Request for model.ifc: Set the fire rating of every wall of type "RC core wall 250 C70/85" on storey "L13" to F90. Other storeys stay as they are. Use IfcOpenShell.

First a look at what the model holds.

```python
import ifcopenshell
import ifcopenshell.util.element

model = ifcopenshell.open("model.ifc")
print(model.schema)
storey = next(s for s in model.by_type("IfcBuildingStorey") if s.Name == "L13")
walls = [e for e in ifcopenshell.util.element.get_decomposition(storey) if e.is_a("IfcWall")]
seen = {}
for e in walls:
    element_type = ifcopenshell.util.element.get_type(e)
    key = (element_type.Name if element_type != e and element_type else None, ifcopenshell.util.element.get_pset(e, "Pset_WallCommon", "FireRating"))
    seen[key] = seen.get(key, 0) + 1
for (name, value), count in sorted(seen.items(), key=str):
    print(count, "x", name, "|", value)
```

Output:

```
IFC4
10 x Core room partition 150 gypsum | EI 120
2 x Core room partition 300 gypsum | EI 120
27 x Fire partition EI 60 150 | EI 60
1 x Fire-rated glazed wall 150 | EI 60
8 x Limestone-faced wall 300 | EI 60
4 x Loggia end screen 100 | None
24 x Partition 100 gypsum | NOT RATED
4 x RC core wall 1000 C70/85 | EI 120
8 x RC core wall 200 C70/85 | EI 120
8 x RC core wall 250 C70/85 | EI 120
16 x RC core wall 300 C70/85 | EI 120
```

```python
import ifcopenshell
import ifcopenshell.api.pset
import ifcopenshell.util.element

model = ifcopenshell.open("model.ifc")

storey = next(s for s in model.by_type("IfcBuildingStorey") if s.Name == "L13")
walls = [e for e in ifcopenshell.util.element.get_decomposition(storey) if e.is_a("IfcWall")]

count = 0
for e in walls:
    element_type = ifcopenshell.util.element.get_type(e)
    if element_type in (None, e) or element_type.Name != "RC core wall 250 C70/85":
        continue
    found = ifcopenshell.util.element.get_pset(e, "Pset_WallCommon", should_inherit=False)
    if found:
        pset = model.by_id(found["id"])
        if len(ifcopenshell.util.element.get_elements_by_pset(pset)) > 1:
            pset = ifcopenshell.api.pset.unshare_pset(model, products=[e], pset=pset)[0]
    else:
        pset = ifcopenshell.api.pset.add_pset(model, product=e, name="Pset_WallCommon")
    ifcopenshell.api.pset.edit_pset(model, pset=pset, properties={"FireRating": "F90"})
    count += 1

print(count, "walls updated")

model.write("model_updated.ifc")
```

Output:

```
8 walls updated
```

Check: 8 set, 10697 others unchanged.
